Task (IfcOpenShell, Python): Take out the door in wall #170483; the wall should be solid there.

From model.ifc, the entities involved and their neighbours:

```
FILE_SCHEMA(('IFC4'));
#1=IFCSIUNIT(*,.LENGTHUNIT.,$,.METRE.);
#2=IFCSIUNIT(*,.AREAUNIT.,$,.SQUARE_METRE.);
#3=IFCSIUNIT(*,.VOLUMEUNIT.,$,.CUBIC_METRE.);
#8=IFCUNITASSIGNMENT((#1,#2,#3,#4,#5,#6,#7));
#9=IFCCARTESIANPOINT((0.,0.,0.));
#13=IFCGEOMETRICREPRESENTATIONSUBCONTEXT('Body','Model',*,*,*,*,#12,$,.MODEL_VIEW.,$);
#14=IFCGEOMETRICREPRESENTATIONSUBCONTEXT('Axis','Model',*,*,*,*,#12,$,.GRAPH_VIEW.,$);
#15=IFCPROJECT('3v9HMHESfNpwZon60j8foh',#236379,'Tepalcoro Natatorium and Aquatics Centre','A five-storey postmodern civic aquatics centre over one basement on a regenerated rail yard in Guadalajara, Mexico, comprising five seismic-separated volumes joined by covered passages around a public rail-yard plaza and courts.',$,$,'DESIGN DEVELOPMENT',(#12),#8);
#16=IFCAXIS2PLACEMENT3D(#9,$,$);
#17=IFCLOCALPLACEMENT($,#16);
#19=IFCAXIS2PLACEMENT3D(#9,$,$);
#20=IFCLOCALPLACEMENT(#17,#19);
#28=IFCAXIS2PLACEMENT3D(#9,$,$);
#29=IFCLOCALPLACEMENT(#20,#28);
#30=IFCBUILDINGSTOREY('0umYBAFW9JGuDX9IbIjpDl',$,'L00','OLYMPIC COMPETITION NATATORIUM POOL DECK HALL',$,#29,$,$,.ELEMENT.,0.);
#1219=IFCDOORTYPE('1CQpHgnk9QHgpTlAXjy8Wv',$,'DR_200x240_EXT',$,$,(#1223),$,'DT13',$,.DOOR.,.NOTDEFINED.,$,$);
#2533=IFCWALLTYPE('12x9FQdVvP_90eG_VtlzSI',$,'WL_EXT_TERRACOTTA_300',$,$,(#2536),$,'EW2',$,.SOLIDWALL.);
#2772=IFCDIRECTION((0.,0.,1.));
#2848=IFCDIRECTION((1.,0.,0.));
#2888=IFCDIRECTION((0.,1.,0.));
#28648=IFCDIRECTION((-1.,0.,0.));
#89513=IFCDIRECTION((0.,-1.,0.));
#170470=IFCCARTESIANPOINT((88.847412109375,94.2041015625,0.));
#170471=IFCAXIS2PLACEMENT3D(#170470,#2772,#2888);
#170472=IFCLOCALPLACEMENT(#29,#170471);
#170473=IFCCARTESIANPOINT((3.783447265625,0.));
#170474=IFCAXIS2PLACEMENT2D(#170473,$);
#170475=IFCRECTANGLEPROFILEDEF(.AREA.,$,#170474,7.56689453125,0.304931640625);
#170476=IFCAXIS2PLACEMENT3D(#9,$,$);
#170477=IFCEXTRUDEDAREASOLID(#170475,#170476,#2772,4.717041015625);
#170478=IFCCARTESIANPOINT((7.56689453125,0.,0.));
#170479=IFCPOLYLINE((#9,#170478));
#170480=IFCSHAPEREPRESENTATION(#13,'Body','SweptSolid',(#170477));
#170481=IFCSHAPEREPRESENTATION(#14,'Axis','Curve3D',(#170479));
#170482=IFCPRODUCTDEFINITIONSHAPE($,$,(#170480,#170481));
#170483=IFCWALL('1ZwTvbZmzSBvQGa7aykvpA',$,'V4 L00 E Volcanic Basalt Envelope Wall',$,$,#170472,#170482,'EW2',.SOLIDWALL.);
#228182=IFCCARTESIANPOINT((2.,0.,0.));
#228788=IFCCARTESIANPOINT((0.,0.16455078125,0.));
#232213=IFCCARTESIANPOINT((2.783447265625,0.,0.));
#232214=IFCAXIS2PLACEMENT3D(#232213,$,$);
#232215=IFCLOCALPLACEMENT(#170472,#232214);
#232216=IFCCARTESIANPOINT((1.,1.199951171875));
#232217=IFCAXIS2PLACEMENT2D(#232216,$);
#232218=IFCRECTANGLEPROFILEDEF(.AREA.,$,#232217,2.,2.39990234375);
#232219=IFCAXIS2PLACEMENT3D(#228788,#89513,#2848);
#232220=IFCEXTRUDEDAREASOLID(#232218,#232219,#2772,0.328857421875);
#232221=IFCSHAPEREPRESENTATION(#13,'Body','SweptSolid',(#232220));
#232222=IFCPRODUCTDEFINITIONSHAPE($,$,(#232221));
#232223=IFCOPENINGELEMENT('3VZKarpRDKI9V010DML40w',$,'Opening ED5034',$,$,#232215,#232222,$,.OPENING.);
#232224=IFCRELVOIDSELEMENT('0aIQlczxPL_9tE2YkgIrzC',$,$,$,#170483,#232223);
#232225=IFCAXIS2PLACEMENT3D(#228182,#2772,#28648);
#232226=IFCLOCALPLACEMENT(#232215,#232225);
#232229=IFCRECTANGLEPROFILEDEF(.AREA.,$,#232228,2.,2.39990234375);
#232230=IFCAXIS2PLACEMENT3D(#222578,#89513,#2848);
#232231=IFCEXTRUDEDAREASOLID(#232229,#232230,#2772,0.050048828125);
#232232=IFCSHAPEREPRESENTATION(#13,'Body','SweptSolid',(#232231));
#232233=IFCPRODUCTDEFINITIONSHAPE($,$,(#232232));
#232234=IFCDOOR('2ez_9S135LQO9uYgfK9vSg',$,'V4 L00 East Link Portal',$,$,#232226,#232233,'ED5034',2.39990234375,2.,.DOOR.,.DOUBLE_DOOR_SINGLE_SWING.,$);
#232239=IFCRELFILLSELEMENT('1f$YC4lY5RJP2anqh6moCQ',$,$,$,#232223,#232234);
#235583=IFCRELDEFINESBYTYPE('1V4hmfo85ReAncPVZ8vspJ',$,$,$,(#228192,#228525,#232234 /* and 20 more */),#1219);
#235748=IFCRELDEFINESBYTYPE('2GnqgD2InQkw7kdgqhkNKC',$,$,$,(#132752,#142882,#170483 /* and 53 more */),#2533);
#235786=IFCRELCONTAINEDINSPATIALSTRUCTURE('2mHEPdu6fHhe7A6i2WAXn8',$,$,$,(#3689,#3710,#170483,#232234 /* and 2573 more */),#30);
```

```python
import ifcopenshell
import ifcopenshell.api.feature
import ifcopenshell.api.root
import ifcopenshell.geom
import ifcopenshell.util.shape

model = ifcopenshell.open("model.ifc")
settings = ifcopenshell.geom.settings()


def volume(element):
    """Net volume in cubic metres, openings subtracted."""
    shape = ifcopenshell.geom.create_shape(settings, element)
    return ifcopenshell.util.shape.get_volume(shape.geometry)


door = model.by_id(232234)
opening = door.FillsVoids[0].RelatingOpeningElement
wall = opening.VoidsElements[0].RelatingBuildingElement
before = volume(wall)

ifcopenshell.api.root.remove_product(model, product=door)
ifcopenshell.api.feature.remove_feature(model, feature=opening)

after = volume(wall)

print(f"wall volume {before:.3f} -> {after:.3f} m3")

model.write("model_edited.ifc")
```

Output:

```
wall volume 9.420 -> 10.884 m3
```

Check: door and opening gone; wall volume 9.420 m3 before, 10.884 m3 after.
